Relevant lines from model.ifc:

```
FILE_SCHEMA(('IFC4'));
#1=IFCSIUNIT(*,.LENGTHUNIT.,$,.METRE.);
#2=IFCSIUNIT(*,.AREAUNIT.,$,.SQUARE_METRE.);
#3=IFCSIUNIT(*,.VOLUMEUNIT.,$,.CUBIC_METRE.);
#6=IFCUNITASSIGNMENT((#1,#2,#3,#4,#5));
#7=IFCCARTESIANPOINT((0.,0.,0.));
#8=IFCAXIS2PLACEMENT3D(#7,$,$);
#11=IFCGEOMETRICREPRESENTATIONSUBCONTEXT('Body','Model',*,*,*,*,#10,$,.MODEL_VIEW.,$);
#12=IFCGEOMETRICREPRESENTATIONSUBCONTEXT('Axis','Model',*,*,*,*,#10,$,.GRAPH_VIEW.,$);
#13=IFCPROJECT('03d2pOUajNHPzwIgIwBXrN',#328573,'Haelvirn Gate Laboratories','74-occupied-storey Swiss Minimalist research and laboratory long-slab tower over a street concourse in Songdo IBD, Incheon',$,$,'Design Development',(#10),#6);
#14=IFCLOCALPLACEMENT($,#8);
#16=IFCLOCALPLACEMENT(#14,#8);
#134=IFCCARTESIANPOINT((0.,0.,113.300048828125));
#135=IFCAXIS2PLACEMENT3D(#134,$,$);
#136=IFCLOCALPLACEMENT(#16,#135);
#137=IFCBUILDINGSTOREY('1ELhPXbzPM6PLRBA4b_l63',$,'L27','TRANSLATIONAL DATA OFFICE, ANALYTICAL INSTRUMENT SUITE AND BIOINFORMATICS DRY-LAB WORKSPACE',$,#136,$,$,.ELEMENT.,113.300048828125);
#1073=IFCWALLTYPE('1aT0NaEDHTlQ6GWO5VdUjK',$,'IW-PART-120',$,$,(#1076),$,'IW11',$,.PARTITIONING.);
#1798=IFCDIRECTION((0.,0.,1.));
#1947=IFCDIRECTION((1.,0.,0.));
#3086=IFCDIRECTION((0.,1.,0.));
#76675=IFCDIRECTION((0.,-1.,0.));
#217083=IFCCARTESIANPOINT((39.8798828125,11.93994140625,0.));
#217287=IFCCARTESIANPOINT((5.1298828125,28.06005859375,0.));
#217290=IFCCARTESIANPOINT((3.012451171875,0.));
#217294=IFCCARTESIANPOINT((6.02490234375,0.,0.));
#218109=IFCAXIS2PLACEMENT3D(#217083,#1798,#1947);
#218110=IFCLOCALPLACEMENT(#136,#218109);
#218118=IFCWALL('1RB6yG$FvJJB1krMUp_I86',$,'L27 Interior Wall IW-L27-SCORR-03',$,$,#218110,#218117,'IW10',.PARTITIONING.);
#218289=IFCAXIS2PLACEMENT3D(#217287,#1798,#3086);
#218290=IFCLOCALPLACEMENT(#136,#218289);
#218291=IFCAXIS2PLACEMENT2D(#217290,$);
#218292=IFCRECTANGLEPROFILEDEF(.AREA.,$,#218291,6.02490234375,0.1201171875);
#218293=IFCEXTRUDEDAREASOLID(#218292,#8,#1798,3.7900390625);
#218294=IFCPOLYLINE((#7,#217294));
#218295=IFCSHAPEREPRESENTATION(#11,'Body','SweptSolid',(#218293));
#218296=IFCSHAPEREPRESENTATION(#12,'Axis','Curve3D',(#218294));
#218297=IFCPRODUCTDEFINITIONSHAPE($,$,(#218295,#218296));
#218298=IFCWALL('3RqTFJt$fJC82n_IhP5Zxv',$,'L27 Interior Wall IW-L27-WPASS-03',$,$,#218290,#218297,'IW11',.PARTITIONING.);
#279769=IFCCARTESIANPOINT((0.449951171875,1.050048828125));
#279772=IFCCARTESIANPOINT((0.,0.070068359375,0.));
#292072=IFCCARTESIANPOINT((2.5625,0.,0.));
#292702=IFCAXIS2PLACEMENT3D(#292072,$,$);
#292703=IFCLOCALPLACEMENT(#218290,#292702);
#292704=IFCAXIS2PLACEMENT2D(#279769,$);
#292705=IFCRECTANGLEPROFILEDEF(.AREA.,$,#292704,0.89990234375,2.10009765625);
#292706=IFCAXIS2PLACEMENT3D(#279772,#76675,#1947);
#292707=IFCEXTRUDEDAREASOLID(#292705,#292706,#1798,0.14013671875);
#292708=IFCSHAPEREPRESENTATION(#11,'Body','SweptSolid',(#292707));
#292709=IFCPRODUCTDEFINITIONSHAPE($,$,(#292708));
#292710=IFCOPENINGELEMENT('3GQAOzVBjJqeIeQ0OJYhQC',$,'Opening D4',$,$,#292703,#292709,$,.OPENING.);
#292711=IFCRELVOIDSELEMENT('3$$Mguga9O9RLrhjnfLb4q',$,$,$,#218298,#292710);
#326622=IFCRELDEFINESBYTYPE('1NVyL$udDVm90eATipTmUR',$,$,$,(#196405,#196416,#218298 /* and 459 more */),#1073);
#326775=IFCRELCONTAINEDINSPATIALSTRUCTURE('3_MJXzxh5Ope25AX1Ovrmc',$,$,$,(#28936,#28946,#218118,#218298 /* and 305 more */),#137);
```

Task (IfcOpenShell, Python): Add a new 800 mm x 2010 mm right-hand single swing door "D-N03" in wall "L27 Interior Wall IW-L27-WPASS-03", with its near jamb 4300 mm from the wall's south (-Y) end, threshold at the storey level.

```python
import numpy as np
import ifcopenshell
import ifcopenshell.api.feature
import ifcopenshell.api.geometry
import ifcopenshell.api.root
import ifcopenshell.api.spatial
import ifcopenshell.geom
import ifcopenshell.util.element
import ifcopenshell.util.placement
import ifcopenshell.util.representation
import ifcopenshell.util.shape
import ifcopenshell.util.unit

model = ifcopenshell.open("model.ifc")
unit_scale = ifcopenshell.util.unit.calculate_unit_scale(model)
settings = ifcopenshell.geom.settings()


def volume(element):
    """Net volume in cubic metres, openings subtracted."""
    shape = ifcopenshell.geom.create_shape(settings, element)
    return ifcopenshell.util.shape.get_volume(shape.geometry)


wall = model.by_guid("3RqTFJt$fJC82n_IhP5Zxv")
storey = ifcopenshell.util.element.get_container(wall, ifc_class="IfcBuildingStorey")
context = ifcopenshell.util.representation.get_context(model, "Model", "Body", "MODEL_VIEW")
before = volume(wall)

width, height, from_end, sill = 0.8, 2.01, 4.3, 0.0  # metres

# The wall runs along its own X axis, and the end named is its -X end.
wall_shape = ifcopenshell.geom.create_shape(settings, wall)
x, y, z = ifcopenshell.util.shape.get_vertices(wall_shape.geometry).T
start = x.min() + from_end
face, thickness = float(y.min()), float(y.max() - y.min())
wall_matrix = ifcopenshell.util.placement.get_local_placement(wall.ObjectPlacement)
level = ifcopenshell.util.placement.get_local_placement(storey.ObjectPlacement)[2, 3]


def in_wall(x, y):
    """Placement at x, y metres in the wall's axes, at sill height."""
    matrix = wall_matrix.copy()
    matrix[:, 3] = wall_matrix @ np.array([x / unit_scale, y / unit_scale, 0.0, 1.0])
    matrix[2, 3] = level + sill / unit_scale
    return matrix


# Opening: a box that overshoots both wall faces by 50 mm.
opening = ifcopenshell.api.root.create_entity(model, ifc_class="IfcOpeningElement", predefined_type="OPENING")
box = ifcopenshell.api.geometry.add_wall_representation(
    model, context=context, length=width, height=height, thickness=thickness + 0.1
)
ifcopenshell.api.geometry.assign_representation(model, product=opening, representation=box)
ifcopenshell.api.geometry.edit_object_placement(model, product=opening, matrix=in_wall(start, face - 0.05), is_si=False)
ifcopenshell.api.feature.add_feature(model, feature=opening, element=wall)

door = ifcopenshell.api.root.create_entity(model, ifc_class="IfcDoor", name="D-N03", predefined_type="DOOR")
door.OverallWidth, door.OverallHeight = width / unit_scale, height / unit_scale
door.OperationType = "SINGLE_SWING_RIGHT"
body = ifcopenshell.api.geometry.add_door_representation(
    model,
    context=context,
    overall_width=door.OverallWidth,
    overall_height=door.OverallHeight,
    operation_type="SINGLE_SWING_RIGHT",
    lining_properties={"LiningDepth": thickness / unit_scale, "ThresholdDepth": thickness / unit_scale},
)
ifcopenshell.api.geometry.assign_representation(model, product=door, representation=body)
ifcopenshell.api.spatial.assign_container(model, products=[door], relating_structure=storey)
ifcopenshell.api.feature.add_filling(model, opening=opening, element=door)

# The lining spans the wall, so the door starts at the wall face.
ifcopenshell.api.geometry.edit_object_placement(model, product=door, matrix=in_wall(start, face), is_si=False)

after = volume(wall)

print(f"wall volume {before:.3f} -> {after:.3f} m3")

model.write("model-out.ifc")
```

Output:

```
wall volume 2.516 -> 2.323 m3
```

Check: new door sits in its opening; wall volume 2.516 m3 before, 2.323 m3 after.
